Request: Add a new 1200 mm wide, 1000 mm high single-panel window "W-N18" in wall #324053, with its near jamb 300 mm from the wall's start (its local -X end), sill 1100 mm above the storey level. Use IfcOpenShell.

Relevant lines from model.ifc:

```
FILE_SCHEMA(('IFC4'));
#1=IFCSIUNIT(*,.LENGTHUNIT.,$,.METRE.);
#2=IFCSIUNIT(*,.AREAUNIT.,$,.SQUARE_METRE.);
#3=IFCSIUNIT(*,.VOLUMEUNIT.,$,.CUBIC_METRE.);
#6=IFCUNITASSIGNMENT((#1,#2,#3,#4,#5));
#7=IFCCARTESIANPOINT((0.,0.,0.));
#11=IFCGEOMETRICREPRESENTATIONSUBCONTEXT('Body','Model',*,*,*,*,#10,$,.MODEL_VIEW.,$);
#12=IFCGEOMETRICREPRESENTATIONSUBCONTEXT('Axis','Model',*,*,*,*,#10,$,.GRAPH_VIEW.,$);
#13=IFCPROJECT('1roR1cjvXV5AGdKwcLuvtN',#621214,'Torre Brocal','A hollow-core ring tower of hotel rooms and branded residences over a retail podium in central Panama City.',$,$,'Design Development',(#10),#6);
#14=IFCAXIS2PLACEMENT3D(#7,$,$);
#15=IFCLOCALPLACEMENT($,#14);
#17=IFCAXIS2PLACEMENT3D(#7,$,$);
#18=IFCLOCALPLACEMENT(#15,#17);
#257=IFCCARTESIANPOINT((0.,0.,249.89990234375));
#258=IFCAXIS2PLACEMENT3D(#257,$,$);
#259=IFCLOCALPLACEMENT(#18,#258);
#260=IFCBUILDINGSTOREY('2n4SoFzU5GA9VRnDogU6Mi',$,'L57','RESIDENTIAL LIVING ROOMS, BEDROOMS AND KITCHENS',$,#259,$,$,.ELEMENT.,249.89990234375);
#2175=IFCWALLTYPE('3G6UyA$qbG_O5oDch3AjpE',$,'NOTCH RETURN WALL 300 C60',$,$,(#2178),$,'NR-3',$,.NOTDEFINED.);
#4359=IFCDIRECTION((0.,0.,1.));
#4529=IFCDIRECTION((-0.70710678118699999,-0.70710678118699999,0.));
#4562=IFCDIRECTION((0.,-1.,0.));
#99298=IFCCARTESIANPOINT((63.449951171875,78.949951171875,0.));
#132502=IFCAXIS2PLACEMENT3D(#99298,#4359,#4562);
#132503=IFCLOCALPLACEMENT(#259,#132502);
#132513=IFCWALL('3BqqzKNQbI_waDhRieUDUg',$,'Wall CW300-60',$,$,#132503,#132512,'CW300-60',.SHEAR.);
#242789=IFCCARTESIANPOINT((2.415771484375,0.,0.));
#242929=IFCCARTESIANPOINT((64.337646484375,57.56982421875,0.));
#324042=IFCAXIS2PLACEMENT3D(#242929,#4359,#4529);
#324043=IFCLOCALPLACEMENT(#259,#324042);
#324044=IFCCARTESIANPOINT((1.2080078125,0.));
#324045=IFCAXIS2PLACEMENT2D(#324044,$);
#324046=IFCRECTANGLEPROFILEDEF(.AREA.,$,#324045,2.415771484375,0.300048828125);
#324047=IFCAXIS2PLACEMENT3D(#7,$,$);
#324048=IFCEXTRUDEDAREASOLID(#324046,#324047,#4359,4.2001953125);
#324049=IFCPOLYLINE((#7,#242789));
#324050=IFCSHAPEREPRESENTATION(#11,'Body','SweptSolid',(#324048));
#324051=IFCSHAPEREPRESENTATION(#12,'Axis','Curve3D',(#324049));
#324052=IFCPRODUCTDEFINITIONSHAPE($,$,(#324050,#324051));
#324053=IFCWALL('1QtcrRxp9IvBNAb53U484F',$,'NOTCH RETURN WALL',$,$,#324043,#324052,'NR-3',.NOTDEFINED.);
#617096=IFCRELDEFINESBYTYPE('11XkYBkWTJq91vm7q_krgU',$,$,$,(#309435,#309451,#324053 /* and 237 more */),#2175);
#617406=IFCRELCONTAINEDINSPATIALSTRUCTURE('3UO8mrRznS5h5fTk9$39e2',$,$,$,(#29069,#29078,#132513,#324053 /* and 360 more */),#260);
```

```python
import numpy as np
import ifcopenshell
import ifcopenshell.api.feature
import ifcopenshell.api.geometry
import ifcopenshell.api.root
import ifcopenshell.api.spatial
import ifcopenshell.geom
import ifcopenshell.util.element
import ifcopenshell.util.placement
import ifcopenshell.util.representation
import ifcopenshell.util.shape
import ifcopenshell.util.unit

model = ifcopenshell.open("model.ifc")
unit_scale = ifcopenshell.util.unit.calculate_unit_scale(model)
settings = ifcopenshell.geom.settings()


def volume(element):
    """Net volume in cubic metres, openings subtracted."""
    shape = ifcopenshell.geom.create_shape(settings, element)
    return ifcopenshell.util.shape.get_volume(shape.geometry)


wall = model.by_guid("1QtcrRxp9IvBNAb53U484F")
storey = ifcopenshell.util.element.get_container(wall, ifc_class="IfcBuildingStorey")
context = ifcopenshell.util.representation.get_context(model, "Model", "Body", "MODEL_VIEW")
before = volume(wall)

width, height, from_end, sill = 1.2, 1, 0.3, 1.1  # metres

# The wall runs along its own X axis, and the end named is its -X end.
wall_shape = ifcopenshell.geom.create_shape(settings, wall)
x, y, z = ifcopenshell.util.shape.get_vertices(wall_shape.geometry).T
start = x.min() + from_end
face, thickness = float(y.min()), float(y.max() - y.min())
wall_matrix = ifcopenshell.util.placement.get_local_placement(wall.ObjectPlacement)
level = ifcopenshell.util.placement.get_local_placement(storey.ObjectPlacement)[2, 3]


def in_wall(x, y):
    """Placement at x, y metres in the wall's axes, at sill height."""
    matrix = wall_matrix.copy()
    matrix[:, 3] = wall_matrix @ np.array([x / unit_scale, y / unit_scale, 0.0, 1.0])
    matrix[2, 3] = level + sill / unit_scale
    return matrix


# Opening: a box that overshoots both wall faces by 50 mm.
opening = ifcopenshell.api.root.create_entity(model, ifc_class="IfcOpeningElement", predefined_type="OPENING")
box = ifcopenshell.api.geometry.add_wall_representation(
    model, context=context, length=width, height=height, thickness=thickness + 0.1
)
ifcopenshell.api.geometry.assign_representation(model, product=opening, representation=box)
ifcopenshell.api.geometry.edit_object_placement(model, product=opening, matrix=in_wall(start, face - 0.05), is_si=False)
ifcopenshell.api.feature.add_feature(model, feature=opening, element=wall)

window = ifcopenshell.api.root.create_entity(model, ifc_class="IfcWindow", name="W-N18", predefined_type="WINDOW")
window.OverallWidth, window.OverallHeight = width / unit_scale, height / unit_scale
window.PartitioningType = "SINGLE_PANEL"
body = ifcopenshell.api.geometry.add_window_representation(
    model,
    context=context,
    overall_width=window.OverallWidth,
    overall_height=window.OverallHeight,
    partition_type="SINGLE_PANEL",
)
ifcopenshell.api.geometry.assign_representation(model, product=window, representation=body)
ifcopenshell.api.spatial.assign_container(model, products=[window], relating_structure=storey)
ifcopenshell.api.feature.add_filling(model, opening=opening, element=window)

# Centre the window in the wall's thickness.
ifcopenshell.api.geometry.edit_object_placement(model, product=window, matrix=in_wall(start, face), is_si=False)
window_shape = ifcopenshell.geom.create_shape(settings, window)
depth = ifcopenshell.util.shape.get_vertices(window_shape.geometry)[:, 1]
offset = face + thickness / 2 - (depth.min() + depth.max()) / 2
ifcopenshell.api.geometry.edit_object_placement(model, product=window, matrix=in_wall(start, offset), is_si=False)

after = volume(wall)

print(f"wall volume {before:.3f} -> {after:.3f} m3")

model.write("model_v2.ifc")
```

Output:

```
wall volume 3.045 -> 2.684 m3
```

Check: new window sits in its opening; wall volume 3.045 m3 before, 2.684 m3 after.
